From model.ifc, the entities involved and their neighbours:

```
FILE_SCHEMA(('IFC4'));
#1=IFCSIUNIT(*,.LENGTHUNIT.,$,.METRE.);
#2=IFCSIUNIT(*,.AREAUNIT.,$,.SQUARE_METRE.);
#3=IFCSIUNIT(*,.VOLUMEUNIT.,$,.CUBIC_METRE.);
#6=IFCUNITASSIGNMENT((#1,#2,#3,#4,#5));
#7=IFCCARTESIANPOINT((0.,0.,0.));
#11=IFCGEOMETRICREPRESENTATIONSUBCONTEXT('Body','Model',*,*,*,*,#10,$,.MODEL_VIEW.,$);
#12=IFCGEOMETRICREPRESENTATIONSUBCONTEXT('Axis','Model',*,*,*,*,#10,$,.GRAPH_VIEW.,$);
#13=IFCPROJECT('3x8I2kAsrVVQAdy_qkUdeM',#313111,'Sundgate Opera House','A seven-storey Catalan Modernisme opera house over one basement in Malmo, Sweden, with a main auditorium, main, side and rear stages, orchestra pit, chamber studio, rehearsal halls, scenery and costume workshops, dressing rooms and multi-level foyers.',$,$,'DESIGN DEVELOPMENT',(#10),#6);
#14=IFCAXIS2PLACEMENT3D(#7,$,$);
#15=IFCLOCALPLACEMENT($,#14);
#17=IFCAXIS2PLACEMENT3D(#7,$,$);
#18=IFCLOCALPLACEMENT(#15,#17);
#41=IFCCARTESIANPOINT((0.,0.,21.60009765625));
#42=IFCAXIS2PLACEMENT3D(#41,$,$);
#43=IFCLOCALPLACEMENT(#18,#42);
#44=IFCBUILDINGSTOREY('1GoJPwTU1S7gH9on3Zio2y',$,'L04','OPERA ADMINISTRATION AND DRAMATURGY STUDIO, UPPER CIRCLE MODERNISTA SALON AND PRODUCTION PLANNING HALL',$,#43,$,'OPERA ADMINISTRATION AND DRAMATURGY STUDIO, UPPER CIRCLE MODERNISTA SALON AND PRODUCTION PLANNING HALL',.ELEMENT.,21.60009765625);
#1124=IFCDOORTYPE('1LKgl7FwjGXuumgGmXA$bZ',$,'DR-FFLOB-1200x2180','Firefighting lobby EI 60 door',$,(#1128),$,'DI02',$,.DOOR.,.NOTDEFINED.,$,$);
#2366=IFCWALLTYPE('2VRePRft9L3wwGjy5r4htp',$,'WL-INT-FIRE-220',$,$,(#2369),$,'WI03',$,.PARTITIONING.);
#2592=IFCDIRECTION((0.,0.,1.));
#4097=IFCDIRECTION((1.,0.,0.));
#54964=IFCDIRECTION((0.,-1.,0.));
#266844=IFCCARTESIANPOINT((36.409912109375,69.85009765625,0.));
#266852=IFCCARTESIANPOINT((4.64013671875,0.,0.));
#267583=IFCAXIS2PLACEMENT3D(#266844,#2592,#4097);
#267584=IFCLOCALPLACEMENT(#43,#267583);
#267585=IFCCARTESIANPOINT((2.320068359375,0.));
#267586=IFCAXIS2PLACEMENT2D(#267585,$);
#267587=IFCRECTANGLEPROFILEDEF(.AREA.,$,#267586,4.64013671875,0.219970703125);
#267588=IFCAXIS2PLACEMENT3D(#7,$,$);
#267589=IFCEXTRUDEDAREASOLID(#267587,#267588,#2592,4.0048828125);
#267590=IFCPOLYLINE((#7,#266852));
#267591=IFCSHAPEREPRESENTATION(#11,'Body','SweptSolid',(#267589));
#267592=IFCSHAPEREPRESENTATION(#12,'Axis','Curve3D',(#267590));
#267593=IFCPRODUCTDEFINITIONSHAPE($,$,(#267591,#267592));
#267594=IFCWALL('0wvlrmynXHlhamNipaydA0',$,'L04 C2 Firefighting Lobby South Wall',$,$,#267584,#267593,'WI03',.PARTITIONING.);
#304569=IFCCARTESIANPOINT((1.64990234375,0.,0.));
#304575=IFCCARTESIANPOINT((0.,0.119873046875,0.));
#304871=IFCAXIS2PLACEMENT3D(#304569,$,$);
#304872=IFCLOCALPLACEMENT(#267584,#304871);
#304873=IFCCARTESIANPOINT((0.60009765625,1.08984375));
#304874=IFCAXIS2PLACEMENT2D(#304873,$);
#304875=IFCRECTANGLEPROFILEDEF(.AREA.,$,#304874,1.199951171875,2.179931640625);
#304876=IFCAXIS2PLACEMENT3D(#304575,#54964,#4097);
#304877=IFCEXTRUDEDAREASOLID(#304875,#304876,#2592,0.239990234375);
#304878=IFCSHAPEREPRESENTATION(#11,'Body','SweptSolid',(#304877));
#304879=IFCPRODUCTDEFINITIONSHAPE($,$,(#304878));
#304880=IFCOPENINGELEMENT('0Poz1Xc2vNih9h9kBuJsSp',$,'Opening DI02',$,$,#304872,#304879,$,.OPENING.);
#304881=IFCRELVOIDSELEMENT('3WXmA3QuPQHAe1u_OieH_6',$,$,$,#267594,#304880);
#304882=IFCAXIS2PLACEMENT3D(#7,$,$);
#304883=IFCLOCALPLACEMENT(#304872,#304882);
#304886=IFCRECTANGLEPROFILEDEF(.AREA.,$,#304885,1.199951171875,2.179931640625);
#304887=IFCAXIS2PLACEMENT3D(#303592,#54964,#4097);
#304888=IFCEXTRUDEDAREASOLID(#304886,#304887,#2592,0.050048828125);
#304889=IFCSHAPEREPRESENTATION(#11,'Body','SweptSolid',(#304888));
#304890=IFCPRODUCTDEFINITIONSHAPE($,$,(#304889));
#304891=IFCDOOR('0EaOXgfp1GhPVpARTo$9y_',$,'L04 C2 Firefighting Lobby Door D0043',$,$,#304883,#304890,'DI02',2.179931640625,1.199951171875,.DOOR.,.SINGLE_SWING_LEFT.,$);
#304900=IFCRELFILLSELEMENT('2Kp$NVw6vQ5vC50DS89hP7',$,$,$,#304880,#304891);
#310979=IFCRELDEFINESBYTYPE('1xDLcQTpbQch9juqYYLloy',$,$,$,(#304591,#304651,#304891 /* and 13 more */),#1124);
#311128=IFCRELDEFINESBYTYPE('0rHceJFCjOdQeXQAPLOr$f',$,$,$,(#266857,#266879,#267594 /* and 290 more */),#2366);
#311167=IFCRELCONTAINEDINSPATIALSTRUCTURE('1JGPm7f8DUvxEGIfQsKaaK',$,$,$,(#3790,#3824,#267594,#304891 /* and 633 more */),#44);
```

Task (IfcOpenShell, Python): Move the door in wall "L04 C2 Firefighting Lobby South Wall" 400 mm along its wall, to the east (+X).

```python
import ifcopenshell
import ifcopenshell.api.geometry
import ifcopenshell.util.placement

model = ifcopenshell.open("model.ifc")

door = model.by_guid("0EaOXgfp1GhPVpARTo$9y_")
opening = door.FillsVoids[0].RelatingOpeningElement
wall = opening.VoidsElements[0].RelatingBuildingElement

wall_matrix = ifcopenshell.util.placement.get_local_placement(wall.ObjectPlacement)
shift = wall_matrix[:3, 0] * 0.4
before = ifcopenshell.util.placement.get_local_placement(door.ObjectPlacement)[:3, 3].copy()

# The door is placed relative to its opening, so it follows when the opening moves.
matrix = ifcopenshell.util.placement.get_local_placement(opening.ObjectPlacement)
matrix[:3, 3] += shift
ifcopenshell.api.geometry.edit_object_placement(
    model, product=opening, matrix=matrix, is_si=False, should_transform_children=True
)

after = ifcopenshell.util.placement.get_local_placement(door.ObjectPlacement)[:3, 3]
print("door moved by", (after - before).round(3) + 0.0)

model.write("model_rev.ifc")
```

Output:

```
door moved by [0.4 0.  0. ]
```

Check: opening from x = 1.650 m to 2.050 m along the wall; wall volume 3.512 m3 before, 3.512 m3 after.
